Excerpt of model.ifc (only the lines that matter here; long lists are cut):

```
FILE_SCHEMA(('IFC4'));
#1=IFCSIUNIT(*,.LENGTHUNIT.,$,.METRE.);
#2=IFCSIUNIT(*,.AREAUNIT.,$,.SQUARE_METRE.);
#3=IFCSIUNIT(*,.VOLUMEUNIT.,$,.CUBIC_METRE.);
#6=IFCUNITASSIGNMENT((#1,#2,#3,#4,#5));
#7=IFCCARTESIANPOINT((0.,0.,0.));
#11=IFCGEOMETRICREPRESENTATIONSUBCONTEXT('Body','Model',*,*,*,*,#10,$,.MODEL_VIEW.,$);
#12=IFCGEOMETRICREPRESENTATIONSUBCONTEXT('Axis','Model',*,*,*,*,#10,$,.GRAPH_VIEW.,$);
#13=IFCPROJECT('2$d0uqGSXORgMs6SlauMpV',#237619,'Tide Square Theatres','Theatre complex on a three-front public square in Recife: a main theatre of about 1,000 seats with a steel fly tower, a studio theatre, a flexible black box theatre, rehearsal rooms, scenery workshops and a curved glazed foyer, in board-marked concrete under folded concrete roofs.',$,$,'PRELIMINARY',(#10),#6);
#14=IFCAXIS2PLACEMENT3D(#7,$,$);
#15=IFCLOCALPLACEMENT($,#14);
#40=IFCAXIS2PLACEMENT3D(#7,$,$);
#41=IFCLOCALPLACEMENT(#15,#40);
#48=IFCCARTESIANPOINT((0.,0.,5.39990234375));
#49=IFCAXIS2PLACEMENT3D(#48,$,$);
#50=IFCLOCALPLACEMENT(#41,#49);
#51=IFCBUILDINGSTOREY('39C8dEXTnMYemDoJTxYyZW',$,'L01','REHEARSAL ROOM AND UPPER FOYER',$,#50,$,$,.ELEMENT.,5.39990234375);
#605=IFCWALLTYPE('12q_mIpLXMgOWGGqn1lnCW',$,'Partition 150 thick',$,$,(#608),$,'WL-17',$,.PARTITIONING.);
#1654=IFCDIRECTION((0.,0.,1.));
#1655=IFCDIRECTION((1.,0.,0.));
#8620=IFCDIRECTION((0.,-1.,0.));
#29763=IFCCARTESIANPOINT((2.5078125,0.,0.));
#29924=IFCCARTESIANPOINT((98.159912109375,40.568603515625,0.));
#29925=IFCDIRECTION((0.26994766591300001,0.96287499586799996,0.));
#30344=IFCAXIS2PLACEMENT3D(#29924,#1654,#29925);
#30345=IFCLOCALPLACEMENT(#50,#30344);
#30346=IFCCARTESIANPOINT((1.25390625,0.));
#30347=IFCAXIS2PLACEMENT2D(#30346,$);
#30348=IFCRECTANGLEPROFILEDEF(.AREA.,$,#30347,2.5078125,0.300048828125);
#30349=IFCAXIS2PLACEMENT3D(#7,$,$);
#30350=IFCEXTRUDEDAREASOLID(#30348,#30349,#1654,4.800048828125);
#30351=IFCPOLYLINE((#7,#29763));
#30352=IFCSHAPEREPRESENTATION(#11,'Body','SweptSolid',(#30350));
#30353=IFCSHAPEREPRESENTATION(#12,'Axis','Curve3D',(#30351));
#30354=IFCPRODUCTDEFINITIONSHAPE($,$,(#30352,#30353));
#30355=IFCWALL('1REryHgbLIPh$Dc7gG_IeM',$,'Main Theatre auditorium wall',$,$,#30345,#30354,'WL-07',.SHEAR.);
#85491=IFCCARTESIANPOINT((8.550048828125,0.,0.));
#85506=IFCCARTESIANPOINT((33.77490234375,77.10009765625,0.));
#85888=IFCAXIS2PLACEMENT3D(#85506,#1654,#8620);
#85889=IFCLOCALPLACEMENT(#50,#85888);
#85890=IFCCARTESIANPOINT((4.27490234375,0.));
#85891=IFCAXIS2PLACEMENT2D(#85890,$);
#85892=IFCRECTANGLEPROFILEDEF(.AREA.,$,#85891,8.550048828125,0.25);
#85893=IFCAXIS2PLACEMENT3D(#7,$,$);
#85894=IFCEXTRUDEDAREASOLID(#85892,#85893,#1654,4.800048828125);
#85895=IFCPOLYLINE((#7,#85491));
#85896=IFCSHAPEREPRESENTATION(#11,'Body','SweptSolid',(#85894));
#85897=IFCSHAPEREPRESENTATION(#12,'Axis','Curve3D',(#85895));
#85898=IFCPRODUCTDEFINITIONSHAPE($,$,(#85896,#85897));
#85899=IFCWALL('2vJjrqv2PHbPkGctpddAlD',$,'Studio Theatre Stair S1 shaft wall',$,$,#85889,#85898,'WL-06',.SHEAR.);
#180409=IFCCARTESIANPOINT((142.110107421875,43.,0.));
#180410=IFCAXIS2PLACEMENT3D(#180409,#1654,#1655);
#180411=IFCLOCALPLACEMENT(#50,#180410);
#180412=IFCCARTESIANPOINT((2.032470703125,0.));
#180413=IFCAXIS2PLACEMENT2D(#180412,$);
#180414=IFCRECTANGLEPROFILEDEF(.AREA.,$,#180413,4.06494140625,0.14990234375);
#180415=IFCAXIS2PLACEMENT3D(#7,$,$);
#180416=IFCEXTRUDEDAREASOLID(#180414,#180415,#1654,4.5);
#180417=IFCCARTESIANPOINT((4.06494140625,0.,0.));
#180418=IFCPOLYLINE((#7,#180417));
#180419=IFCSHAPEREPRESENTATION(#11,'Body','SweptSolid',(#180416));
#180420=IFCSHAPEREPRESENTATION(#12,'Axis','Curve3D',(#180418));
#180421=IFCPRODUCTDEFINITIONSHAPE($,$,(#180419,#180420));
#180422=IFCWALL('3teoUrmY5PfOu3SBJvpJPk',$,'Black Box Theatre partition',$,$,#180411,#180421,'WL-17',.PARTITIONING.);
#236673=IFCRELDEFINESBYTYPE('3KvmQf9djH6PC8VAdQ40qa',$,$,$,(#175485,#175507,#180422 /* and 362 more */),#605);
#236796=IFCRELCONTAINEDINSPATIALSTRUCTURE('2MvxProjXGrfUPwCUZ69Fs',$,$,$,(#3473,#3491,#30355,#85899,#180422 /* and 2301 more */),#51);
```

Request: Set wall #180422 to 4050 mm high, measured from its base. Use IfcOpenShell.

```python
import ifcopenshell
import ifcopenshell.geom
import ifcopenshell.util.representation
import ifcopenshell.util.shape

model = ifcopenshell.open("model.ifc")
settings = ifcopenshell.geom.settings()


def volume(element):
    """Net volume in cubic metres, openings subtracted."""
    shape = ifcopenshell.geom.create_shape(settings, element)
    return ifcopenshell.util.shape.get_volume(shape.geometry)


wall = model.by_guid("3teoUrmY5PfOu3SBJvpJPk")
before = volume(wall)

body = ifcopenshell.util.representation.get_representation(wall, "Model", "Body")
solid = body.Items[0]
old_height = solid.Depth
solid.Depth = 4.05
after = volume(wall)

print(f"height {old_height:g} -> {solid.Depth:g}, volume {before:.3f} -> {after:.3f} m3")

model.write("model_rev.ifc")
```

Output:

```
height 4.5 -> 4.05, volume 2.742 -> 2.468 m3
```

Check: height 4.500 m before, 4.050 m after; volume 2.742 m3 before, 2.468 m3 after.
